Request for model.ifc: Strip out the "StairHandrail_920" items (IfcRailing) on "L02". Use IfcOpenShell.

First a look at what the model holds.

```python
import ifcopenshell
import ifcopenshell.util.element

model = ifcopenshell.open("model.ifc")
print(model.schema)
storey = next(s for s in model.by_type("IfcBuildingStorey") if s.Name == "L02")
railings = [e for e in ifcopenshell.util.element.get_decomposition(storey) if e.is_a("IfcRailing")]
seen = {}
for e in railings:
    element_type = ifcopenshell.util.element.get_type(e)
    name = element_type.Name if element_type not in (None, e) else None
    seen[name] = seen.get(name, 0) + 1
for name, count in sorted(seen.items(), key=str):
    print(count, "x", name)
```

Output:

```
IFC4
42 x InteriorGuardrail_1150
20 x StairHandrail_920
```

```python
import ifcopenshell
import ifcopenshell.api.root
import ifcopenshell.util.element

model = ifcopenshell.open("model.ifc")

storey = next(s for s in model.by_type("IfcBuildingStorey") if s.Name == "L02")
railings = [e for e in ifcopenshell.util.element.get_decomposition(storey) if e.is_a("IfcRailing")]
targets = [e for e in railings if (t := ifcopenshell.util.element.get_type(e)) not in (None, e) and t.Name == "StairHandrail_920"]

for e in targets:
    ifcopenshell.api.root.remove_product(model, product=e)
print(len(targets), "removed")

model.write("model_edited.ifc")
```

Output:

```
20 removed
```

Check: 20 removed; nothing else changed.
